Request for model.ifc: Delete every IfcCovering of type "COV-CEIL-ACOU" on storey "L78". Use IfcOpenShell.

First a look at what the model holds.

```python
import ifcopenshell
import ifcopenshell.util.element

model = ifcopenshell.open("model.ifc")
print(model.schema)
storey = next(s for s in model.by_type("IfcBuildingStorey") if s.Name == "L78")
coverings = [e for e in ifcopenshell.util.element.get_decomposition(storey) if e.is_a("IfcCovering")]
seen = {}
for e in coverings:
    element_type = ifcopenshell.util.element.get_type(e)
    name = element_type.Name if element_type not in (None, e) else None
    seen[name] = seen.get(name, 0) + 1
for name, count in sorted(seen.items(), key=str):
    print(count, "x", name)
```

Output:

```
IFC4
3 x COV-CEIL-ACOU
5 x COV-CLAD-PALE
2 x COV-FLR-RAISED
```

```python
import ifcopenshell
import ifcopenshell.api.root
import ifcopenshell.util.element

model = ifcopenshell.open("model.ifc")

storey = next(s for s in model.by_type("IfcBuildingStorey") if s.Name == "L78")
coverings = [e for e in ifcopenshell.util.element.get_decomposition(storey) if e.is_a("IfcCovering")]
targets = [e for e in coverings if (t := ifcopenshell.util.element.get_type(e)) not in (None, e) and t.Name == "COV-CEIL-ACOU"]

for e in targets:
    ifcopenshell.api.root.remove_product(model, product=e)
print(len(targets), "removed")

model.write("model_v2.ifc")
```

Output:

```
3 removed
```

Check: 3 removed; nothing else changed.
